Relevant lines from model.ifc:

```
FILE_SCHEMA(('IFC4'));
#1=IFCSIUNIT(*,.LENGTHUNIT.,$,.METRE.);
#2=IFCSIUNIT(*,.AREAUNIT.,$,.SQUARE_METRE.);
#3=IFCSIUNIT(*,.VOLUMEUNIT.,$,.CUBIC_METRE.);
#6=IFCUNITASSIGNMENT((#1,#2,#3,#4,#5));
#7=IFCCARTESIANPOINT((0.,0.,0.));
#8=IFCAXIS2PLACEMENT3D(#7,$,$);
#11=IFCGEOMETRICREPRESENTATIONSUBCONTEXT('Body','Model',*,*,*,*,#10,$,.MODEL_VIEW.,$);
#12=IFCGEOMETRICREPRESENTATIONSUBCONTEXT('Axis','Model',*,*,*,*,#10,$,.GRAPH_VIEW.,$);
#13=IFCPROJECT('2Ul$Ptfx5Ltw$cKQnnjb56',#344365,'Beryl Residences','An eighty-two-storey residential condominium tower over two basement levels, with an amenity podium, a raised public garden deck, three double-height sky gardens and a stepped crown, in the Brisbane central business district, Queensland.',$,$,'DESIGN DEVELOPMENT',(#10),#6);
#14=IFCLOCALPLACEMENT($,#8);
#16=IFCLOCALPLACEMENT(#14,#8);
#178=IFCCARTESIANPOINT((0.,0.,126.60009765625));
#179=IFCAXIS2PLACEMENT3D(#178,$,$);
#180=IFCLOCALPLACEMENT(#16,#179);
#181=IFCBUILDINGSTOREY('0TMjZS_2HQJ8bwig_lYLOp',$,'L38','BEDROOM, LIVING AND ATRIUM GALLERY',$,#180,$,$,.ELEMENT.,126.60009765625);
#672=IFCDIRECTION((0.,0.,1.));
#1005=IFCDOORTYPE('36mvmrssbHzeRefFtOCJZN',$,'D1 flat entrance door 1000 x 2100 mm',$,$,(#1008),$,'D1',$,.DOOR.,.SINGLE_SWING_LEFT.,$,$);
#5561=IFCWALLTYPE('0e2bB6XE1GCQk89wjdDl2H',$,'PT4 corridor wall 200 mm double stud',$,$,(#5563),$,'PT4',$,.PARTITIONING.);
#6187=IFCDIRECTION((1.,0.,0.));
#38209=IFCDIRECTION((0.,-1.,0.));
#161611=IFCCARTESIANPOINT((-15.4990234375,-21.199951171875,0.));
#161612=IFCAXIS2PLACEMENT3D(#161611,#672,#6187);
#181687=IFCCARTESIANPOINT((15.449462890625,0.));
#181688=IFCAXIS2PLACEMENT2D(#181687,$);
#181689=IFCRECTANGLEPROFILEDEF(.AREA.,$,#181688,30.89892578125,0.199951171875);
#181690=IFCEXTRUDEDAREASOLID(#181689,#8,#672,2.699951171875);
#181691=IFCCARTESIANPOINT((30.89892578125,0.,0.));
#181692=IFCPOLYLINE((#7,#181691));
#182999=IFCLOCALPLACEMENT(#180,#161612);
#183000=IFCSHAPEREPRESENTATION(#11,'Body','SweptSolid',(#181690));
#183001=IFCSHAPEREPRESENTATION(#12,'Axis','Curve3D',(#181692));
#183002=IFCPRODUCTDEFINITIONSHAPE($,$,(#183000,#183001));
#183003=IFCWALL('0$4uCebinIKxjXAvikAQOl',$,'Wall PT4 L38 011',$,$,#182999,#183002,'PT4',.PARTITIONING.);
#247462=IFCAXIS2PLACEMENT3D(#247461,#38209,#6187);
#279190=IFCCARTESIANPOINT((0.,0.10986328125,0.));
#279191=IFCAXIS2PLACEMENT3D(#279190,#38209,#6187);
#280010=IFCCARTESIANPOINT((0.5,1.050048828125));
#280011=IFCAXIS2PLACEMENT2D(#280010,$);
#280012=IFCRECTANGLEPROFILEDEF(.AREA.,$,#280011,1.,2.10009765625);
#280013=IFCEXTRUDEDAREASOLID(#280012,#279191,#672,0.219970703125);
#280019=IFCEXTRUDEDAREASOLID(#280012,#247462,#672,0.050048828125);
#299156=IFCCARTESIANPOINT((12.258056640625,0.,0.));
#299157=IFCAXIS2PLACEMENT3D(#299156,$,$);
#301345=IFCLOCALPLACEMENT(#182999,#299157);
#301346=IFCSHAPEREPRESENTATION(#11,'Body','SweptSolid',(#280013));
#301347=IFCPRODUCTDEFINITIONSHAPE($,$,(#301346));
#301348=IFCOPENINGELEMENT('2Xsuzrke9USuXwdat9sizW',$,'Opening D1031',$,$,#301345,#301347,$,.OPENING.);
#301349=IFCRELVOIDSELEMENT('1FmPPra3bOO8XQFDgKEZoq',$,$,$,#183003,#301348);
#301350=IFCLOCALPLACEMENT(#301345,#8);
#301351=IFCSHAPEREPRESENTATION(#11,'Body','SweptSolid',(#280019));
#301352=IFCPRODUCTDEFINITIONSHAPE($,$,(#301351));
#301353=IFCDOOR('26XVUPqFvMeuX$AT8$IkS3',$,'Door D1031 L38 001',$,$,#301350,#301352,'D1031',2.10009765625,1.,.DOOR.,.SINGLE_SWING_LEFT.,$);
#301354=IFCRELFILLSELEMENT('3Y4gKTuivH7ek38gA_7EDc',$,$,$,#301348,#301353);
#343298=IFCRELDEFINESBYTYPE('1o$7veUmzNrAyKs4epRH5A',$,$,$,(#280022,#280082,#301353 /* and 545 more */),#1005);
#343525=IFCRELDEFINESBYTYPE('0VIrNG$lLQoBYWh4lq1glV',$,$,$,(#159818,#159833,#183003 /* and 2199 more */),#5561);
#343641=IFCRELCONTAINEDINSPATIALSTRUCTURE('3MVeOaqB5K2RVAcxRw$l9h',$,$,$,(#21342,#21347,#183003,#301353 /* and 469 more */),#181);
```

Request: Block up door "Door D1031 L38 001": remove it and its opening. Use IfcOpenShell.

```python
import ifcopenshell
import ifcopenshell.api.feature
import ifcopenshell.api.root
import ifcopenshell.geom
import ifcopenshell.util.shape

model = ifcopenshell.open("model.ifc")
settings = ifcopenshell.geom.settings()


def volume(element):
    """Net volume in cubic metres, openings subtracted."""
    shape = ifcopenshell.geom.create_shape(settings, element)
    return ifcopenshell.util.shape.get_volume(shape.geometry)


door = model.by_guid("26XVUPqFvMeuX$AT8$IkS3")
opening = door.FillsVoids[0].RelatingOpeningElement
wall = opening.VoidsElements[0].RelatingBuildingElement
before = volume(wall)

ifcopenshell.api.root.remove_product(model, product=door)
ifcopenshell.api.feature.remove_feature(model, feature=opening)

after = volume(wall)

print(f"wall volume {before:.3f} -> {after:.3f} m3")

model.write("model_edited.ifc")
```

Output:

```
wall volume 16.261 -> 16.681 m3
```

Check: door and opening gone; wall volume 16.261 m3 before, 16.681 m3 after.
